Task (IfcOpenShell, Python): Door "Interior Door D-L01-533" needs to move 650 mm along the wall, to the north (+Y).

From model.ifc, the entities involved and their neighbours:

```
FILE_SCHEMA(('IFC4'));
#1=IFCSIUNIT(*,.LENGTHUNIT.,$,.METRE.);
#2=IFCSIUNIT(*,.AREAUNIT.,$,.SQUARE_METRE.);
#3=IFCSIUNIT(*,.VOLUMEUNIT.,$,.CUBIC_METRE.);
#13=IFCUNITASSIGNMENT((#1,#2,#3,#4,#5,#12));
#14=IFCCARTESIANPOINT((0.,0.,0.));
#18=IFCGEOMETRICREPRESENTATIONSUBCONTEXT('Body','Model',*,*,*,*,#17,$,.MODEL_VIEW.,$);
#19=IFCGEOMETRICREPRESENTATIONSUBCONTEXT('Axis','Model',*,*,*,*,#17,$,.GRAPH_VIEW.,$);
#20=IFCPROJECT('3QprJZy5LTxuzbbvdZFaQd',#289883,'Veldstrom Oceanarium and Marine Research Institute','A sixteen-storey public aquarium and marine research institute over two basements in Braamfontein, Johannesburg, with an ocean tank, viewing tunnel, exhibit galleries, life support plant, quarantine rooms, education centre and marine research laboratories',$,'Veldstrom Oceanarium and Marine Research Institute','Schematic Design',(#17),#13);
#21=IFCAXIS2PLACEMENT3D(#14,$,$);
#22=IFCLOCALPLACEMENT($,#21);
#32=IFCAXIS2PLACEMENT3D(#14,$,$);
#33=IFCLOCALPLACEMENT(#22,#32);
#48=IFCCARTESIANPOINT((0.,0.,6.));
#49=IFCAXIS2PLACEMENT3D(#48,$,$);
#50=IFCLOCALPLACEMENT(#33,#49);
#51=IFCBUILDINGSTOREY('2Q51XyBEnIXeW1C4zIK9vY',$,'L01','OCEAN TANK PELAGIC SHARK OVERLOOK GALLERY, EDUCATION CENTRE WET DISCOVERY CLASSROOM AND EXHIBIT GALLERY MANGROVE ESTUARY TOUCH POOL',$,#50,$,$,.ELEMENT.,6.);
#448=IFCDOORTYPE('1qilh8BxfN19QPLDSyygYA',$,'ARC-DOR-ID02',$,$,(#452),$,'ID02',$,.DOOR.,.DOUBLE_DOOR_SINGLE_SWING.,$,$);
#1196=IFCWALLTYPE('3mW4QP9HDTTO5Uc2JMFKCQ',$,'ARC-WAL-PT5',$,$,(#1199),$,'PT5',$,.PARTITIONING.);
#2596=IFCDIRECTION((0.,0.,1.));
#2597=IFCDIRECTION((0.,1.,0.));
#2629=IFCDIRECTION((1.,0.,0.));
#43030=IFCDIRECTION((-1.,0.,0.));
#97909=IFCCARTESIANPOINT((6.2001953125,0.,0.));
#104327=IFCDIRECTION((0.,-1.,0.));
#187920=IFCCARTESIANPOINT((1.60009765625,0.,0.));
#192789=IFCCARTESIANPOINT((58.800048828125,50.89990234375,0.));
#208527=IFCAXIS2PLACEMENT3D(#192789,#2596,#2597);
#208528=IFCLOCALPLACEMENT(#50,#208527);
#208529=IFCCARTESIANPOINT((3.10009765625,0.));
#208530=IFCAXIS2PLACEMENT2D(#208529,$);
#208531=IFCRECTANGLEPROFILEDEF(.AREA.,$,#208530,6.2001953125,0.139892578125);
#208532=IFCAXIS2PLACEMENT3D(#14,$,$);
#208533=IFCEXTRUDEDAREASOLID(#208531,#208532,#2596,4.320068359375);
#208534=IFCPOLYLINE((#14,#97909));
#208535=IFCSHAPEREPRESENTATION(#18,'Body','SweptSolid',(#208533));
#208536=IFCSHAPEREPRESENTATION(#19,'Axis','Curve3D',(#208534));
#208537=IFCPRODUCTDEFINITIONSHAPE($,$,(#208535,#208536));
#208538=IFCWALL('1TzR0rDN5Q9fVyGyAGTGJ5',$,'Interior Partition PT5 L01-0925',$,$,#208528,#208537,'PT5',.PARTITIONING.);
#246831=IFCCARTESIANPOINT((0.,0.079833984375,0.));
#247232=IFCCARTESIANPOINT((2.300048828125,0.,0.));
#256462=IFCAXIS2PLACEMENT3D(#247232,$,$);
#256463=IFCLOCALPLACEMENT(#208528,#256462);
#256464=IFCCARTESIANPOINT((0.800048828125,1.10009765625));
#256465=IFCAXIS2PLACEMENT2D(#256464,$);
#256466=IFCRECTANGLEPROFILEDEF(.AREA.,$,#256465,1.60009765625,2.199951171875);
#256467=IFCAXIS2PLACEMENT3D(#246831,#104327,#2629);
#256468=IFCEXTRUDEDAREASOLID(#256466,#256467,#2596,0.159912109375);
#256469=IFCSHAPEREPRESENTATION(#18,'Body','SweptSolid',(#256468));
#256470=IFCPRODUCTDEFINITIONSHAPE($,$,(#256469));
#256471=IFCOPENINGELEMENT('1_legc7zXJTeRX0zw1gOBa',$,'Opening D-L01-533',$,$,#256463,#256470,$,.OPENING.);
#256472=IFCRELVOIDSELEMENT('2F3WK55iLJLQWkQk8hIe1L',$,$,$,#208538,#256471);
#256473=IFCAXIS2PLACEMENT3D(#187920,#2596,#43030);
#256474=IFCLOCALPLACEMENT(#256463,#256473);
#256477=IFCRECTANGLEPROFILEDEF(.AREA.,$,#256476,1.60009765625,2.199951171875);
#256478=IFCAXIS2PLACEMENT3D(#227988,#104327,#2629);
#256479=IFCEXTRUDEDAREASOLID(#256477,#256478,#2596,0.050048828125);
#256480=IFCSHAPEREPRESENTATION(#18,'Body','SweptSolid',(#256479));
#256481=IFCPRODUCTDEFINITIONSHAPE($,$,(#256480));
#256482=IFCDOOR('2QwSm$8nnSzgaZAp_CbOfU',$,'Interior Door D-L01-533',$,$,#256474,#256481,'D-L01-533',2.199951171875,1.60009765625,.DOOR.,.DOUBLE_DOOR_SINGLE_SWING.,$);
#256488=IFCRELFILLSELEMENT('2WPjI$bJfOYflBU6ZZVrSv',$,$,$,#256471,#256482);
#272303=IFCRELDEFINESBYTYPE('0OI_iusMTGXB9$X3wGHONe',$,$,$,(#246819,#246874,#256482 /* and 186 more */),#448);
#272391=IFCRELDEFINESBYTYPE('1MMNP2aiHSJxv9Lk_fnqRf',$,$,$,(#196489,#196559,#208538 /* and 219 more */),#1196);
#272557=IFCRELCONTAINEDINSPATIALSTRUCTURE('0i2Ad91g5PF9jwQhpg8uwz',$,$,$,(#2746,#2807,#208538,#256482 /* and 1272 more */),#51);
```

```python
import ifcopenshell
import ifcopenshell.api.geometry
import ifcopenshell.util.placement
import ifcopenshell.util.unit

model = ifcopenshell.open("model.ifc")
unit_scale = ifcopenshell.util.unit.calculate_unit_scale(model)

door = model.by_guid("2QwSm$8nnSzgaZAp_CbOfU")
opening = door.FillsVoids[0].RelatingOpeningElement
wall = opening.VoidsElements[0].RelatingBuildingElement

wall_matrix = ifcopenshell.util.placement.get_local_placement(wall.ObjectPlacement)
shift = wall_matrix[:3, 0] * 0.65 / unit_scale
before = ifcopenshell.util.placement.get_local_placement(door.ObjectPlacement)[:3, 3].copy()

# The door is placed relative to its opening, so it follows when the opening moves.
matrix = ifcopenshell.util.placement.get_local_placement(opening.ObjectPlacement)
matrix[:3, 3] += shift
ifcopenshell.api.geometry.edit_object_placement(
    model, product=opening, matrix=matrix, is_si=False, should_transform_children=True
)

after = ifcopenshell.util.placement.get_local_placement(door.ObjectPlacement)[:3, 3]
print("door moved by", (after - before).round(3) + 0.0)

model.write("model_updated.ifc")
```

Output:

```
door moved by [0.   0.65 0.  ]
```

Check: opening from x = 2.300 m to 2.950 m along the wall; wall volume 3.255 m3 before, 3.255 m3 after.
